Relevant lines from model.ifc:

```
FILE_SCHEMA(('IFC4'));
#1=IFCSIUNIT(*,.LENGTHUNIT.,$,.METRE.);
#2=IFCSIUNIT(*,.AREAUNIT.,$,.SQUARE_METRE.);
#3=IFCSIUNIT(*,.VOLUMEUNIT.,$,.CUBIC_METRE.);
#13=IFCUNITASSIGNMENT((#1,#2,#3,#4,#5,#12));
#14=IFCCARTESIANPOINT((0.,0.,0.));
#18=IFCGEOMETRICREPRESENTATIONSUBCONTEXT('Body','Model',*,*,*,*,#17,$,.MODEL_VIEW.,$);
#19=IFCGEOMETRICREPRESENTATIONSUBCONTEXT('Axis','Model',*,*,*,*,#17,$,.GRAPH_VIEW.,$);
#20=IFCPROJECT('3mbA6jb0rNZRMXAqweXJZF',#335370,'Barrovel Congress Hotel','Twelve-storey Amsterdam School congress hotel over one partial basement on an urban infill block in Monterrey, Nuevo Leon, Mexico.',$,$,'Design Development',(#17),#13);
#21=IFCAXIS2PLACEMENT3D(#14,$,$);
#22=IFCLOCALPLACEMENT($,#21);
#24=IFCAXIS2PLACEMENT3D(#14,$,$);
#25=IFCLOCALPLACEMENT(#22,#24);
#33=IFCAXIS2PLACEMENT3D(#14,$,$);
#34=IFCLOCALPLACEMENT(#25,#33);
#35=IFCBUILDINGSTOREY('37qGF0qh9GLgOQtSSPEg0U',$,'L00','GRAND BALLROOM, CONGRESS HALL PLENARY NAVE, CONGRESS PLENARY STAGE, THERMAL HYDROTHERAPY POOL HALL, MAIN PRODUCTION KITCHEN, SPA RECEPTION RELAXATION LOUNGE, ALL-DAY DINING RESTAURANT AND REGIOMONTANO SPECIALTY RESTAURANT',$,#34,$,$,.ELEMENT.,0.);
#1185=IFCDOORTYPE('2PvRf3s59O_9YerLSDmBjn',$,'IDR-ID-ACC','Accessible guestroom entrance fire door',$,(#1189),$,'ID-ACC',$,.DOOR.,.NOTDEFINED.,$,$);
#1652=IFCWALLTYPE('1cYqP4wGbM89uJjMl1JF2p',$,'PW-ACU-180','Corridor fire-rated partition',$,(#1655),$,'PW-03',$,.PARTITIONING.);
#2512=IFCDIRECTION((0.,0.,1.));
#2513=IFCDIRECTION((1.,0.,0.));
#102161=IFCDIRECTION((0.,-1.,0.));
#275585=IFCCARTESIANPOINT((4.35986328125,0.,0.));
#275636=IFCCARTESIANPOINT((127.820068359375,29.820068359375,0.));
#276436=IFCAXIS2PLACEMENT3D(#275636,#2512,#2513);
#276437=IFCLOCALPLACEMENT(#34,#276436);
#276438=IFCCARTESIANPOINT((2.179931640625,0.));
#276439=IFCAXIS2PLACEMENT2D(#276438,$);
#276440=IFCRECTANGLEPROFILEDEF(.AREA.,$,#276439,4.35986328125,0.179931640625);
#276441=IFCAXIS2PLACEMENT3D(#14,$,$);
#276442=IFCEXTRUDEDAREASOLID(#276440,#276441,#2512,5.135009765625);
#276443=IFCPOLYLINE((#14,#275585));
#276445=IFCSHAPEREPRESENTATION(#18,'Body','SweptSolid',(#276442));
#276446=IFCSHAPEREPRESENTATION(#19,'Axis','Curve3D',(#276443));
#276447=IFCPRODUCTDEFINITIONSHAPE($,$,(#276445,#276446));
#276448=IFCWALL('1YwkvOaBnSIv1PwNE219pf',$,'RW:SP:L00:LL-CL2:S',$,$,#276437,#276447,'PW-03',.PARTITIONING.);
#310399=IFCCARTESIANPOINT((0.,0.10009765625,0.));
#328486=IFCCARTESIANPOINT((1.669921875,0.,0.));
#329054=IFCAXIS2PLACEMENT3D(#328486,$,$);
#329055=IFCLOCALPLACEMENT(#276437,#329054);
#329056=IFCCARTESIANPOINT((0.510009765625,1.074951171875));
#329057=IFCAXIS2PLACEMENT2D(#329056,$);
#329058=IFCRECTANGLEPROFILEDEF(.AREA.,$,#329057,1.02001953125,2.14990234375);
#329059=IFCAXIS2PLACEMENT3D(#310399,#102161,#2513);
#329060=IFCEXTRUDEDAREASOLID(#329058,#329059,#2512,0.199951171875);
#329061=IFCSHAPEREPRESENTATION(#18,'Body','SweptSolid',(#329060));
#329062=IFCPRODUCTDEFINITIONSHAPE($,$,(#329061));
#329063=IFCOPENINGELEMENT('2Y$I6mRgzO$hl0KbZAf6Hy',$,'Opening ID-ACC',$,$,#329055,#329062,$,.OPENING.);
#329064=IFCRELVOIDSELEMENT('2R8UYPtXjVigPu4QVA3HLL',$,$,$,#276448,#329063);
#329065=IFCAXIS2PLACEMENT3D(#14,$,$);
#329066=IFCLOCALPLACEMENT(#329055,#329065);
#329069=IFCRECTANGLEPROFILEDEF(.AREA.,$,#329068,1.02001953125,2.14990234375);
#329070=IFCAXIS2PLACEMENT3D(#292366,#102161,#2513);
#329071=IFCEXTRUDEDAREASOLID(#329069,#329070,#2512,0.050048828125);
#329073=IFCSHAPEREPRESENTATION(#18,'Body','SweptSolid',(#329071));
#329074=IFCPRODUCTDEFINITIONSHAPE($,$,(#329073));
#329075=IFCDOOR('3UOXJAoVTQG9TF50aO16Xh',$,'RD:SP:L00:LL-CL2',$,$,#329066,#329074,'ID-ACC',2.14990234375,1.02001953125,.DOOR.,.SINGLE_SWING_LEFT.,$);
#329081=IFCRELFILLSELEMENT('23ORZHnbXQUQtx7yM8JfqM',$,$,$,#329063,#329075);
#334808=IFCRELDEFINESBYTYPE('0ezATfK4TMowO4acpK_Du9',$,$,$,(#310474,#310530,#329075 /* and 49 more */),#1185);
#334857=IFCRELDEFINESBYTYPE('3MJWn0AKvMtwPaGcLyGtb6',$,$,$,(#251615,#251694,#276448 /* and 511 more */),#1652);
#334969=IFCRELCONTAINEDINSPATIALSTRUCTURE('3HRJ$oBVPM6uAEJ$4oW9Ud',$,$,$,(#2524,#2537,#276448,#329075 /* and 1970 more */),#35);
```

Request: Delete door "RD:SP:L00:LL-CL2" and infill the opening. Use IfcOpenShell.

```python
import ifcopenshell
import ifcopenshell.api.feature
import ifcopenshell.api.root
import ifcopenshell.geom
import ifcopenshell.util.shape

model = ifcopenshell.open("model.ifc")
settings = ifcopenshell.geom.settings()


def volume(element):
    """Net volume in cubic metres, openings subtracted."""
    shape = ifcopenshell.geom.create_shape(settings, element)
    return ifcopenshell.util.shape.get_volume(shape.geometry)


door = model.by_guid("3UOXJAoVTQG9TF50aO16Xh")
opening = door.FillsVoids[0].RelatingOpeningElement
wall = opening.VoidsElements[0].RelatingBuildingElement
before = volume(wall)

ifcopenshell.api.root.remove_product(model, product=door)
ifcopenshell.api.feature.remove_feature(model, feature=opening)

after = volume(wall)

print(f"wall volume {before:.3f} -> {after:.3f} m3")

model.write("model_edited.ifc")
```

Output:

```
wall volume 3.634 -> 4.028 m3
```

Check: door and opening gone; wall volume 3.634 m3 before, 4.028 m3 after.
